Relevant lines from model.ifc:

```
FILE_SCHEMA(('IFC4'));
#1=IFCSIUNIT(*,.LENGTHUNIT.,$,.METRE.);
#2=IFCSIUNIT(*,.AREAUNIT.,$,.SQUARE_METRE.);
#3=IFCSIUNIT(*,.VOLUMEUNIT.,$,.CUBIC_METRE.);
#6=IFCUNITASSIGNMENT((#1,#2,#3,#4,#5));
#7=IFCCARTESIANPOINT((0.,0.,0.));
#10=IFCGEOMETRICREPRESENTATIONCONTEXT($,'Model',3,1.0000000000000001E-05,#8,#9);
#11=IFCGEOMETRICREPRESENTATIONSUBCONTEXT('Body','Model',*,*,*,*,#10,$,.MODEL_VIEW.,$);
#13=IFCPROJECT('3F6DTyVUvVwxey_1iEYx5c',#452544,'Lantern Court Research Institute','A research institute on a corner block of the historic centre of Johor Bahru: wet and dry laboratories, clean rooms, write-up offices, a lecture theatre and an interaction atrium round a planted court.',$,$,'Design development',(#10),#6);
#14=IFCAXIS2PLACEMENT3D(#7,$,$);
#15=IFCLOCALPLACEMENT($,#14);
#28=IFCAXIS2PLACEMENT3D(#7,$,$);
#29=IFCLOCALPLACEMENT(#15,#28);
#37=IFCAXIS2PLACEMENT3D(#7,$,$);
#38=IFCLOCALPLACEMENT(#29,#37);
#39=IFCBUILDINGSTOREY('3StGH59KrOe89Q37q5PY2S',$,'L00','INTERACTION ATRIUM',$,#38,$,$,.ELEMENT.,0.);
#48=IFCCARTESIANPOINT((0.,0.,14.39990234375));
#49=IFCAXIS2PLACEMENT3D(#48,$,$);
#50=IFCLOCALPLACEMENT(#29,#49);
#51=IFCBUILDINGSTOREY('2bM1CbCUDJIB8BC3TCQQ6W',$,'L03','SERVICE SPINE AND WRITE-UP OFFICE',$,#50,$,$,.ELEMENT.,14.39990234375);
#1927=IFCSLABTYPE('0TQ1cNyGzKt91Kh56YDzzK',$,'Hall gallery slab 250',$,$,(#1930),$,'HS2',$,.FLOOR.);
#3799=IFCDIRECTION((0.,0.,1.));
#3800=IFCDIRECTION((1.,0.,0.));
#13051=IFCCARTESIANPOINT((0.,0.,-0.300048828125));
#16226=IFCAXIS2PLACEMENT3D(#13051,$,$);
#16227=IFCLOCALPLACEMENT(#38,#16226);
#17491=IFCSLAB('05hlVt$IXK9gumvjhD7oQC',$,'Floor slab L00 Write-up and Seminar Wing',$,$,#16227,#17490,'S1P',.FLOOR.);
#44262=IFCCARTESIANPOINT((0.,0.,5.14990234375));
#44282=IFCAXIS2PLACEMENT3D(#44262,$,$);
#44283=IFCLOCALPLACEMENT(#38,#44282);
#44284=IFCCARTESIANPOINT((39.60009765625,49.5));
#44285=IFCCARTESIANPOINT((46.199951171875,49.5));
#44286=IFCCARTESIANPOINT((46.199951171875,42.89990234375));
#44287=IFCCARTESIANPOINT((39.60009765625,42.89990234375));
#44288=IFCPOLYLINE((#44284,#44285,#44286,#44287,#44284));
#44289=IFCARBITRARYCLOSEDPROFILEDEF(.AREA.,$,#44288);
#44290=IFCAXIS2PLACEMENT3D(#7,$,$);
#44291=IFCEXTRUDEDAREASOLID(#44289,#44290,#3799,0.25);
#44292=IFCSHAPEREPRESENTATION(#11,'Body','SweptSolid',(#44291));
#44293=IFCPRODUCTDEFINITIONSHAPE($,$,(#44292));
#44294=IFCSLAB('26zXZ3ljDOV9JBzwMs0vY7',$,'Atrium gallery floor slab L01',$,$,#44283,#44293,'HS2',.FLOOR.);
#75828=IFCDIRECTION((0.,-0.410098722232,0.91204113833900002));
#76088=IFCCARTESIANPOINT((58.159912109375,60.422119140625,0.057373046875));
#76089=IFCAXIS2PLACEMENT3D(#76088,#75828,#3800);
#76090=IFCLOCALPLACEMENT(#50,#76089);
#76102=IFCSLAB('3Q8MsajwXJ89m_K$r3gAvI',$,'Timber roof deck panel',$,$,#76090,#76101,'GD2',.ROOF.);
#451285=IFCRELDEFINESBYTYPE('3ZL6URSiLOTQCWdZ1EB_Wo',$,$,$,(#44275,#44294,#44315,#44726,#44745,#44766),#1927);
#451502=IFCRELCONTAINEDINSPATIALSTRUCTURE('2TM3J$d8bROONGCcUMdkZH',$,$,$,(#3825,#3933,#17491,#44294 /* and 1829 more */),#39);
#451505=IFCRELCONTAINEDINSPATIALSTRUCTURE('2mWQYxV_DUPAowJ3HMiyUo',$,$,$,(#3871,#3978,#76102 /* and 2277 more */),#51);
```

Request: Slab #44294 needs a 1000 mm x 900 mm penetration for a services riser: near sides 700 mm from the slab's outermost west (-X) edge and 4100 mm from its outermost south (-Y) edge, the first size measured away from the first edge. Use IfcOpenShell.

```python
import numpy as np
import ifcopenshell
import ifcopenshell.api.feature
import ifcopenshell.api.geometry
import ifcopenshell.api.root
import ifcopenshell.geom
import ifcopenshell.util.placement
import ifcopenshell.util.representation
import ifcopenshell.util.shape
import ifcopenshell.util.unit

model = ifcopenshell.open("model.ifc")
unit_scale = ifcopenshell.util.unit.calculate_unit_scale(model)
settings = ifcopenshell.geom.settings()


def volume(element):
    """Net volume in cubic metres, openings subtracted."""
    shape = ifcopenshell.geom.create_shape(settings, element)
    return ifcopenshell.util.shape.get_volume(shape.geometry)


slab = model.by_guid("26zXZ3ljDOV9JBzwMs0vY7")
before = volume(slab)

# Extent in the slab's own axes, in metres. The edges named are its -X and -Y sides.
slab_shape = ifcopenshell.geom.create_shape(settings, slab)
vertices = ifcopenshell.util.shape.get_vertices(slab_shape.geometry)
x_min, y_min, bottom = vertices.min(axis=0)
top = vertices[:, 2].max()

opening = ifcopenshell.api.root.create_entity(model, ifc_class="IfcOpeningElement", name="Services riser opening", predefined_type="OPENING")
context = ifcopenshell.util.representation.get_context(model, "Model", "Body", "MODEL_VIEW")
width, depth = 1, 0.9
outline = [(0.0, 0.0), (width, 0.0), (width, depth), (0.0, depth), (0.0, 0.0)]
# Overshoot both faces by 50 mm so the cut is clean.
shape = ifcopenshell.api.geometry.add_slab_representation(
    model, context=context, depth=top - bottom + 0.1, polyline=outline
)
ifcopenshell.api.geometry.assign_representation(model, product=opening, representation=shape)

matrix = ifcopenshell.util.placement.get_local_placement(slab.ObjectPlacement)
matrix[:, 3] = matrix @ np.append(np.array([x_min + 0.7, y_min + 4.1, bottom - 0.05]) / unit_scale, 1.0)
ifcopenshell.api.geometry.edit_object_placement(model, product=opening, matrix=matrix, is_si=False)
ifcopenshell.api.feature.add_feature(model, feature=opening, element=slab)

after = volume(slab)

print(f"slab volume {before:.3f} -> {after:.3f} m3")

model.write("model_rev.ifc")
```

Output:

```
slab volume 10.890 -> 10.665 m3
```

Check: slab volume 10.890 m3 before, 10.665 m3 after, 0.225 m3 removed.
